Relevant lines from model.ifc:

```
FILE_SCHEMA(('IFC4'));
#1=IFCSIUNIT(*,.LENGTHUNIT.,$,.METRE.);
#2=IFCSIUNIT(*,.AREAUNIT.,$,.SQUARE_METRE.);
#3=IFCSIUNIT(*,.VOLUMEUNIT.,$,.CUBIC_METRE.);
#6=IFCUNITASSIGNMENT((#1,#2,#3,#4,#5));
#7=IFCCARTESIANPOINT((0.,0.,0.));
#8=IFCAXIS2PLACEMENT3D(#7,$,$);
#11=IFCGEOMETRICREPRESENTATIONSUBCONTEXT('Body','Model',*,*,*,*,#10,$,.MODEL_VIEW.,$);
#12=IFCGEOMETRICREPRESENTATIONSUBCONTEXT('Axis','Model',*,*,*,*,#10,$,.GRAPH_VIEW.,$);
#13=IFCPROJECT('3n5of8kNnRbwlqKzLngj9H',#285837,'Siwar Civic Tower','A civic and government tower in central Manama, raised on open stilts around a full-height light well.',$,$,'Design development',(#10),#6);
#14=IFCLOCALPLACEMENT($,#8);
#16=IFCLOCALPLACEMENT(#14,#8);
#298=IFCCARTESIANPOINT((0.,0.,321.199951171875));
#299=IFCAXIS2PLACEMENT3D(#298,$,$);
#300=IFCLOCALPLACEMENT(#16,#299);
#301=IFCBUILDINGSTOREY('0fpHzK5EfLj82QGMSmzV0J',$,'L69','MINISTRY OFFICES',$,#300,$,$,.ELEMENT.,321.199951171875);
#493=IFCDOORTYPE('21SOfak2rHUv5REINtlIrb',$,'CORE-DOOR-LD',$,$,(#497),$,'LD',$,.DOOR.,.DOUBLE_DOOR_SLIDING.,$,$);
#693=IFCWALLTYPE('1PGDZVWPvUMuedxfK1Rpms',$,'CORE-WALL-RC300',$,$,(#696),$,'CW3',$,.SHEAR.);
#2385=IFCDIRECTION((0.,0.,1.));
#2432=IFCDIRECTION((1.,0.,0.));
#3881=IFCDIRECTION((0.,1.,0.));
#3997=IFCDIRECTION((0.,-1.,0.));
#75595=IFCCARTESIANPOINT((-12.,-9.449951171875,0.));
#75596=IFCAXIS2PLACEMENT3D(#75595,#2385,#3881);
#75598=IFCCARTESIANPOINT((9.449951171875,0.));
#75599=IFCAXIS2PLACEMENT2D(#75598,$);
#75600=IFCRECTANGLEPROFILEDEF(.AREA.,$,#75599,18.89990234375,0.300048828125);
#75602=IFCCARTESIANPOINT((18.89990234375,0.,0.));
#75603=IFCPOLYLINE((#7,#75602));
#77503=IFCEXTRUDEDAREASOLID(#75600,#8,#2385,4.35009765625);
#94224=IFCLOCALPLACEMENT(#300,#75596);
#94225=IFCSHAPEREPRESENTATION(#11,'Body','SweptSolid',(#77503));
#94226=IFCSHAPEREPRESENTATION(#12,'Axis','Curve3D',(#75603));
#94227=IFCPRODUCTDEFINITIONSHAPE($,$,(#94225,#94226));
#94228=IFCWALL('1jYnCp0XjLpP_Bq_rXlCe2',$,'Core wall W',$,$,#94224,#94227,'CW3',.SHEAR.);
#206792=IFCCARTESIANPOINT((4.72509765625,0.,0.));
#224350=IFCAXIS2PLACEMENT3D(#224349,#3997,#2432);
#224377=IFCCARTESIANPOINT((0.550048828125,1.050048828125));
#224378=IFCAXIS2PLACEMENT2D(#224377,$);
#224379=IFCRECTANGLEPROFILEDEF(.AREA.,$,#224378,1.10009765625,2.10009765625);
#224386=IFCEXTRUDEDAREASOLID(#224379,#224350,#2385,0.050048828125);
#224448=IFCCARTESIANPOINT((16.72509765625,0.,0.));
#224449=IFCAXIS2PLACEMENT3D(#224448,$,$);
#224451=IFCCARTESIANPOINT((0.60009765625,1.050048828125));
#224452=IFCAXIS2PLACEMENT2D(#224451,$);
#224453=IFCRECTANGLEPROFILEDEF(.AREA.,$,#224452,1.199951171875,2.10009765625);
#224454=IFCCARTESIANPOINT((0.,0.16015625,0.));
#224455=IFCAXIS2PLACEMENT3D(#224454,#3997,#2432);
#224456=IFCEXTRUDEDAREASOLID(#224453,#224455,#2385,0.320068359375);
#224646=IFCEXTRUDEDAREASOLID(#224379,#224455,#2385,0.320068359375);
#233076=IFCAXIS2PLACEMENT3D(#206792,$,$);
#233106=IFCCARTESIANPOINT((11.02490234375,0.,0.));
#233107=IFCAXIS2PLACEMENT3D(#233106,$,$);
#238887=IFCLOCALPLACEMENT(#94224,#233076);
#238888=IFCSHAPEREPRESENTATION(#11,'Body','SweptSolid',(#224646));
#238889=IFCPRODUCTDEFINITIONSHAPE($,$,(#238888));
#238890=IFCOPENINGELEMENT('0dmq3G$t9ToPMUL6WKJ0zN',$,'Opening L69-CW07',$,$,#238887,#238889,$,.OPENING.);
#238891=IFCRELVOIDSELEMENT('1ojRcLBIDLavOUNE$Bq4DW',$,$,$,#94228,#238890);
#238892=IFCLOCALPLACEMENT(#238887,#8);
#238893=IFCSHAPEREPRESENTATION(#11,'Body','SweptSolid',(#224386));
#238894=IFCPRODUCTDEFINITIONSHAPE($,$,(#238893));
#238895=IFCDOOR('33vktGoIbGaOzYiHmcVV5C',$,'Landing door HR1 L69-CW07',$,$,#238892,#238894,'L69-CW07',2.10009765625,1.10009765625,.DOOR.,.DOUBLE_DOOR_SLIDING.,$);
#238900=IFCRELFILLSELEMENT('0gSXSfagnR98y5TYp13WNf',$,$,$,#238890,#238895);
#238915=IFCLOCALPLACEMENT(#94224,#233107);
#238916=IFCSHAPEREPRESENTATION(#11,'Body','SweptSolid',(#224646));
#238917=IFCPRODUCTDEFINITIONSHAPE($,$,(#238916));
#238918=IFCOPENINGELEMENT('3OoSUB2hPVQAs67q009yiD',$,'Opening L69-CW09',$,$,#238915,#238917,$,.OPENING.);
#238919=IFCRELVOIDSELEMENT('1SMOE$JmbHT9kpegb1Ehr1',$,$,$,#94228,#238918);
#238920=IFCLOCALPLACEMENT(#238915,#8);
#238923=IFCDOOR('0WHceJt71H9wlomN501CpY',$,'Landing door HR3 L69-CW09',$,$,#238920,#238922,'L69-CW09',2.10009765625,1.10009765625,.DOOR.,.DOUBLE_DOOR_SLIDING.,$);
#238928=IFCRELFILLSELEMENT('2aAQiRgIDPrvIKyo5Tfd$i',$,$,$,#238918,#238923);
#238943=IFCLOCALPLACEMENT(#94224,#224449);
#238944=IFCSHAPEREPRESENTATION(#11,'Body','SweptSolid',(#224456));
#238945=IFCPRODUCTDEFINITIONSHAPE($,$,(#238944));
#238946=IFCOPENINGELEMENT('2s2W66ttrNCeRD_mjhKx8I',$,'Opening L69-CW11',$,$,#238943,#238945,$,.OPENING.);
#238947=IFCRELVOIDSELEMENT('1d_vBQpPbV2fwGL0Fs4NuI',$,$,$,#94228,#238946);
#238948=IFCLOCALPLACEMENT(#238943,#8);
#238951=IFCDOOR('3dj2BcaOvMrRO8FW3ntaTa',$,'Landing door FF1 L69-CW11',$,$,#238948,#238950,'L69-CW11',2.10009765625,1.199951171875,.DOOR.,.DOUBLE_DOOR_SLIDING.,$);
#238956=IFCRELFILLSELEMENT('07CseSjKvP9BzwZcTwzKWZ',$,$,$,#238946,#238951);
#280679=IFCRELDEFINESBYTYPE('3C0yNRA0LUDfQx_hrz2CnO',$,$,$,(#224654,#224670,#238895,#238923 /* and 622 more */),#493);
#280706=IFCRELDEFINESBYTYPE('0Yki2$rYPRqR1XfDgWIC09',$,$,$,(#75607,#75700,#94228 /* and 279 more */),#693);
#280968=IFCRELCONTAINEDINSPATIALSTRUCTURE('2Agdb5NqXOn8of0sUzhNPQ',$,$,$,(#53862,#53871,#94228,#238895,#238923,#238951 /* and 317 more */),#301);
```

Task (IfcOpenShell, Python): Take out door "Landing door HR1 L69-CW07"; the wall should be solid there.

```python
import ifcopenshell
import ifcopenshell.api.feature
import ifcopenshell.api.root
import ifcopenshell.geom
import ifcopenshell.util.shape

model = ifcopenshell.open("model.ifc")
settings = ifcopenshell.geom.settings()


def volume(element):
    """Net volume in cubic metres, openings subtracted."""
    shape = ifcopenshell.geom.create_shape(settings, element)
    return ifcopenshell.util.shape.get_volume(shape.geometry)


door = model.by_id(238895)
opening = door.FillsVoids[0].RelatingOpeningElement
wall = opening.VoidsElements[0].RelatingBuildingElement
before = volume(wall)

ifcopenshell.api.root.remove_product(model, product=door)
ifcopenshell.api.feature.remove_feature(model, feature=opening)

after = volume(wall)

print(f"wall volume {before:.3f} -> {after:.3f} m3")

model.write("model_v2.ifc")
```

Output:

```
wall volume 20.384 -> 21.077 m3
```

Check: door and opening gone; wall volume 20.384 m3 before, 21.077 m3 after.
